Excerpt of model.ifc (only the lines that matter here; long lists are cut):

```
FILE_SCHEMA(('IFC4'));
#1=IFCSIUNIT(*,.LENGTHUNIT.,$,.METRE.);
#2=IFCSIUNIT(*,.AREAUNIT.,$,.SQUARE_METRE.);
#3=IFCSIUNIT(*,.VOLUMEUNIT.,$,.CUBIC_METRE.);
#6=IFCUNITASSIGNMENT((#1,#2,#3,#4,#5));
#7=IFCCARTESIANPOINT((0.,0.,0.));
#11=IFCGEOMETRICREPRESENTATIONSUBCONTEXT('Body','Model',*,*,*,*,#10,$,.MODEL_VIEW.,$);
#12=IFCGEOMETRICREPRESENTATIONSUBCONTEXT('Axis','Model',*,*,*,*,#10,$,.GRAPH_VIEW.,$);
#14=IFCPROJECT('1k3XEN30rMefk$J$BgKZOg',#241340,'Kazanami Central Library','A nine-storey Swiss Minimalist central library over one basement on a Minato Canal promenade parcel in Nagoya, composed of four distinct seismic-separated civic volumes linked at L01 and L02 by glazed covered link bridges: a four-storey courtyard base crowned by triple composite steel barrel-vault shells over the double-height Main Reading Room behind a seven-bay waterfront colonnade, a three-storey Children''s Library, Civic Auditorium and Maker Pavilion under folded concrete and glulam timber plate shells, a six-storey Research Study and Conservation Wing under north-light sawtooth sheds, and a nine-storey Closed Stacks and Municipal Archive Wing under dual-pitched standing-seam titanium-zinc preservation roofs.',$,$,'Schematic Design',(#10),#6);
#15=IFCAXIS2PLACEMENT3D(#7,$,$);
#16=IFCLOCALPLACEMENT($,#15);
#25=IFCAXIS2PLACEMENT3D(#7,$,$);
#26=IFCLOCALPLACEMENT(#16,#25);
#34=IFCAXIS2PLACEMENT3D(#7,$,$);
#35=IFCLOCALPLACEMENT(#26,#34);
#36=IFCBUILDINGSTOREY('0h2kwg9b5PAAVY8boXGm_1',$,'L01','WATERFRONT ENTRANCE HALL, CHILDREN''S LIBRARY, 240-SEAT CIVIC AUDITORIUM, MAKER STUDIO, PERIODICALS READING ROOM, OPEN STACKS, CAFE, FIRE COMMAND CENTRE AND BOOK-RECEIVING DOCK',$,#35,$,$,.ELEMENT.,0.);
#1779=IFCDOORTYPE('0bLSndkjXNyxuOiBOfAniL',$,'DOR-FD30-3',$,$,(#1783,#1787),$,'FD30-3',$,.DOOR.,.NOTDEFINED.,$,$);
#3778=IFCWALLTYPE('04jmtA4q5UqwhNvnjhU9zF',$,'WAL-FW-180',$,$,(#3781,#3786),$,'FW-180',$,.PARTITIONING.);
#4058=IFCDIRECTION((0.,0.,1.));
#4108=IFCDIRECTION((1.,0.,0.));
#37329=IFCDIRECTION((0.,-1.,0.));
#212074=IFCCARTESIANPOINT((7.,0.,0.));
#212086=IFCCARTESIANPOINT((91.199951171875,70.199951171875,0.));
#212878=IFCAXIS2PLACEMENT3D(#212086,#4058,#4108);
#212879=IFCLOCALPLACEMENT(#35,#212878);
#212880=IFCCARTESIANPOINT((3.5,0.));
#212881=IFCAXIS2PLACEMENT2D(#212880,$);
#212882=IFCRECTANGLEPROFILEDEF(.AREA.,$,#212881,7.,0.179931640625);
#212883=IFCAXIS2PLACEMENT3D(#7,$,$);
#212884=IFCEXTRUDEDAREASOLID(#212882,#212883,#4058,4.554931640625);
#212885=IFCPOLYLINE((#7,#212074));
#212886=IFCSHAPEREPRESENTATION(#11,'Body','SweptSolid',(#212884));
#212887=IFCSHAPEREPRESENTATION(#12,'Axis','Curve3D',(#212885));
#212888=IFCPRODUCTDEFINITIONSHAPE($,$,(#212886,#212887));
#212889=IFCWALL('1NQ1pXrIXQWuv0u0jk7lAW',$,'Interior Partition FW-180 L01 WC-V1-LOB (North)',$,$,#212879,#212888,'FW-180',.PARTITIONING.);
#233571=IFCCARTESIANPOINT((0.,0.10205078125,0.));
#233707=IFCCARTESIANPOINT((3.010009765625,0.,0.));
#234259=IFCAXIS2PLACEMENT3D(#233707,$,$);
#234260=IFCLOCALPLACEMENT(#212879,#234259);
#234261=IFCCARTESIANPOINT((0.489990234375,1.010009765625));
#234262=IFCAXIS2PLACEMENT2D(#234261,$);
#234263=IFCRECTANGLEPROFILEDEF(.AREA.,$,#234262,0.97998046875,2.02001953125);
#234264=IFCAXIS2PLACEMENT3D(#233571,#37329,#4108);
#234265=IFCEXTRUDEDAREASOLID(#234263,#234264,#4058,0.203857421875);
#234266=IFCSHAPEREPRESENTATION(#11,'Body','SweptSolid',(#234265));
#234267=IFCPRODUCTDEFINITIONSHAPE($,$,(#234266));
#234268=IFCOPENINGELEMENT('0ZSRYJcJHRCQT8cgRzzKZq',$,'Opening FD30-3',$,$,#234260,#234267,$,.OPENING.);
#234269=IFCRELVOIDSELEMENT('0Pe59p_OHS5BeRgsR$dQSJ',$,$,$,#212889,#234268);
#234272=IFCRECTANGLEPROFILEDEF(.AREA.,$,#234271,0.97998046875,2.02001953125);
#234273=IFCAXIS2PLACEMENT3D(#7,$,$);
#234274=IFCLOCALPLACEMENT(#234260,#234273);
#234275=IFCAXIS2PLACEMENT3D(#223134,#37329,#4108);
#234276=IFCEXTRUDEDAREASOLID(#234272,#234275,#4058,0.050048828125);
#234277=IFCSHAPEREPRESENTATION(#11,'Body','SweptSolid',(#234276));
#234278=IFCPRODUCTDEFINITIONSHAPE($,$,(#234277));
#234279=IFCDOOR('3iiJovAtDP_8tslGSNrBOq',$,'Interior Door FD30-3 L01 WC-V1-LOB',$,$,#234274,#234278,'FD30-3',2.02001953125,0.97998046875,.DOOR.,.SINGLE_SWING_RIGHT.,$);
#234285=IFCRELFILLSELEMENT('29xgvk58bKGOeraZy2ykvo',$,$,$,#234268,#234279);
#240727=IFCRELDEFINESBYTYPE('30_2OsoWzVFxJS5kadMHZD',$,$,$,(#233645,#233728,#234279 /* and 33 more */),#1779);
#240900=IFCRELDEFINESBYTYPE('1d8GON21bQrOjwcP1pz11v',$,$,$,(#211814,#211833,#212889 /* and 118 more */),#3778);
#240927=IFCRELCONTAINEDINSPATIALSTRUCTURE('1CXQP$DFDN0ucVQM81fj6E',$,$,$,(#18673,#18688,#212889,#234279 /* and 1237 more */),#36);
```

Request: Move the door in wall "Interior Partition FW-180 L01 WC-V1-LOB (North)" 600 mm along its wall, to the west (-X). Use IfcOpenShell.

```python
import ifcopenshell
import ifcopenshell.api.geometry
import ifcopenshell.util.placement
import ifcopenshell.util.unit

model = ifcopenshell.open("model.ifc")
unit_scale = ifcopenshell.util.unit.calculate_unit_scale(model)

door = model.by_guid("3iiJovAtDP_8tslGSNrBOq")
opening = door.FillsVoids[0].RelatingOpeningElement
wall = opening.VoidsElements[0].RelatingBuildingElement

wall_matrix = ifcopenshell.util.placement.get_local_placement(wall.ObjectPlacement)
shift = wall_matrix[:3, 0] * -0.6 / unit_scale
before = ifcopenshell.util.placement.get_local_placement(door.ObjectPlacement)[:3, 3].copy()

# The door is placed relative to its opening, so it follows when the opening moves.
matrix = ifcopenshell.util.placement.get_local_placement(opening.ObjectPlacement)
matrix[:3, 3] += shift
ifcopenshell.api.geometry.edit_object_placement(
    model, product=opening, matrix=matrix, is_si=False, should_transform_children=True
)

after = ifcopenshell.util.placement.get_local_placement(door.ObjectPlacement)[:3, 3]
print("door moved by", (after - before).round(3) + 0.0)

model.write("model_rev.ifc")
```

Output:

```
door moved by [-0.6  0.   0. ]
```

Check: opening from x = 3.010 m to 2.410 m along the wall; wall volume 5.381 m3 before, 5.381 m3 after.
